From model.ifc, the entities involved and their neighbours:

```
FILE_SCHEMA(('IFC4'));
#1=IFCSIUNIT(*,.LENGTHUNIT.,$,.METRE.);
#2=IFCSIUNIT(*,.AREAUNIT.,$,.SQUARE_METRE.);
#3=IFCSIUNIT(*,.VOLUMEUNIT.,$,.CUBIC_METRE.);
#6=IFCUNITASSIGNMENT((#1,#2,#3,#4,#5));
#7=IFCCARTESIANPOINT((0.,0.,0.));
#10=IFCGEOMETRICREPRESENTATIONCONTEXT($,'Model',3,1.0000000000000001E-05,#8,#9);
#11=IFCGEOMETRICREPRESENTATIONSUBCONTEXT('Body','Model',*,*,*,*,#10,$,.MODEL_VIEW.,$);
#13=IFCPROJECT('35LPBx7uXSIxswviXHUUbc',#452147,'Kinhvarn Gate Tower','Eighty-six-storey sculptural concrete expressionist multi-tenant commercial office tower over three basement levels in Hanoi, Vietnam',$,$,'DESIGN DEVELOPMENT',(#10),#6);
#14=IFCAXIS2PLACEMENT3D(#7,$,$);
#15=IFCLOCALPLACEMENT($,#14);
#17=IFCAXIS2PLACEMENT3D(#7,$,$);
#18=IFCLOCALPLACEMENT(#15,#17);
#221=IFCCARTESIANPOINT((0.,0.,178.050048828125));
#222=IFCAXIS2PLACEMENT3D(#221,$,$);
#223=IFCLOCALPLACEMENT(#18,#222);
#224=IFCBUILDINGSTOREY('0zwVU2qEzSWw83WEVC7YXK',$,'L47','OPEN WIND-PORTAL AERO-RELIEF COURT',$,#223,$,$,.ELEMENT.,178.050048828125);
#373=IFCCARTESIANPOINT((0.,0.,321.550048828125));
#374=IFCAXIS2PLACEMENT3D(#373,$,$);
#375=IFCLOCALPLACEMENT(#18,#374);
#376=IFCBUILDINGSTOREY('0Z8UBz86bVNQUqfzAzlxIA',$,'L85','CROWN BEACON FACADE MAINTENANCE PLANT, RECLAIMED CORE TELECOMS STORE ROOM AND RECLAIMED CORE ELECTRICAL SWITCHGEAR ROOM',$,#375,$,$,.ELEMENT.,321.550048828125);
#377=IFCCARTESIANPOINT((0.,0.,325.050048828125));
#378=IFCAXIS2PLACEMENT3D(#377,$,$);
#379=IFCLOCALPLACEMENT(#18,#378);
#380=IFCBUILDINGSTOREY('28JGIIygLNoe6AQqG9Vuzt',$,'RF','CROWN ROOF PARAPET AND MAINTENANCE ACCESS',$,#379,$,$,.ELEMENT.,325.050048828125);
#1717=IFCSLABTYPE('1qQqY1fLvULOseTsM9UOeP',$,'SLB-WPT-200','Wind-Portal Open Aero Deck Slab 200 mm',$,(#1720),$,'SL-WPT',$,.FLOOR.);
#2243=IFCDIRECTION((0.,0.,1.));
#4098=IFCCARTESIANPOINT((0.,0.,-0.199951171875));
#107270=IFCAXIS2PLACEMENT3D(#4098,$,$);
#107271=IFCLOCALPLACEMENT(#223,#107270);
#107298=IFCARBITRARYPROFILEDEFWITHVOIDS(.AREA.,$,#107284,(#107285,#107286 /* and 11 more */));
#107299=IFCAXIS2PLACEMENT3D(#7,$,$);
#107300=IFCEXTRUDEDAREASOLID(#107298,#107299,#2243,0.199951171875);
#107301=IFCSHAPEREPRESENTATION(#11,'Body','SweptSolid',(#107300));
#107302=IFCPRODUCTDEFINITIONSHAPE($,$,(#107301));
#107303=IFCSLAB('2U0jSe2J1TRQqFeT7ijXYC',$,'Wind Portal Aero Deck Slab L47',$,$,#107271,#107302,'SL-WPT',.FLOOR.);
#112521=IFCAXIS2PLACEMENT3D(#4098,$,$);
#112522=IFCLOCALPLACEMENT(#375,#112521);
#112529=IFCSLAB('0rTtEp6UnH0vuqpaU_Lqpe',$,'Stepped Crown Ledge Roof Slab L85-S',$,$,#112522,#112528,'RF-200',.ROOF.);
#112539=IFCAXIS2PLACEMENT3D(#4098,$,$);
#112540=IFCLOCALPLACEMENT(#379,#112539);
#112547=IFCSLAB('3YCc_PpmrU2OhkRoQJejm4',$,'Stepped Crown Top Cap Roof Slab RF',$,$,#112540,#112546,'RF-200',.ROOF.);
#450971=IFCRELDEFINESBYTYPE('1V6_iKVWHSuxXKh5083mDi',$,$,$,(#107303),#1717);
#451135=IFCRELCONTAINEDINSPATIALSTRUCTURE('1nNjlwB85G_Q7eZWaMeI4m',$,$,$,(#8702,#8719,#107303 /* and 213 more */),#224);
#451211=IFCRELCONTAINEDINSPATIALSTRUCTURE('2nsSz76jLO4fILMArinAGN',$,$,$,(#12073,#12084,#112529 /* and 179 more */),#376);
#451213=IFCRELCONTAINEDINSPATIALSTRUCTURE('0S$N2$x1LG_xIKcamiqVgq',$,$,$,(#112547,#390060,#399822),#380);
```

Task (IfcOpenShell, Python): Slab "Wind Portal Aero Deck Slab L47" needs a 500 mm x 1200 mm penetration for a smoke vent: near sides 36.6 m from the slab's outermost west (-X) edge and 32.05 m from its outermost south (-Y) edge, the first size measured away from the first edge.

```python
import numpy as np
import ifcopenshell
import ifcopenshell.api.feature
import ifcopenshell.api.geometry
import ifcopenshell.api.root
import ifcopenshell.geom
import ifcopenshell.util.placement
import ifcopenshell.util.representation
import ifcopenshell.util.shape
import ifcopenshell.util.unit

model = ifcopenshell.open("model.ifc")
unit_scale = ifcopenshell.util.unit.calculate_unit_scale(model)
settings = ifcopenshell.geom.settings()


def volume(element):
    """Net volume in cubic metres, openings subtracted."""
    shape = ifcopenshell.geom.create_shape(settings, element)
    return ifcopenshell.util.shape.get_volume(shape.geometry)


slab = model.by_guid("2U0jSe2J1TRQqFeT7ijXYC")
before = volume(slab)

# Extent in the slab's own axes, in metres. The edges named are its -X and -Y sides.
slab_shape = ifcopenshell.geom.create_shape(settings, slab)
vertices = ifcopenshell.util.shape.get_vertices(slab_shape.geometry)
x_min, y_min, bottom = vertices.min(axis=0)
top = vertices[:, 2].max()

opening = ifcopenshell.api.root.create_entity(model, ifc_class="IfcOpeningElement", name="Smoke vent opening", predefined_type="OPENING")
context = ifcopenshell.util.representation.get_context(model, "Model", "Body", "MODEL_VIEW")
width, depth = 0.5, 1.2
outline = [(0.0, 0.0), (width, 0.0), (width, depth), (0.0, depth), (0.0, 0.0)]
# Overshoot both faces by 50 mm so the cut is clean.
shape = ifcopenshell.api.geometry.add_slab_representation(
    model, context=context, depth=top - bottom + 0.1, polyline=outline
)
ifcopenshell.api.geometry.assign_representation(model, product=opening, representation=shape)

matrix = ifcopenshell.util.placement.get_local_placement(slab.ObjectPlacement)
matrix[:, 3] = matrix @ np.append(np.array([x_min + 36.6, y_min + 32.05, bottom - 0.05]) / unit_scale, 1.0)
ifcopenshell.api.geometry.edit_object_placement(model, product=opening, matrix=matrix, is_si=False)
ifcopenshell.api.feature.add_feature(model, feature=opening, element=slab)

after = volume(slab)

print(f"slab volume {before:.3f} -> {after:.3f} m3")

model.write("model_edited.ifc")
```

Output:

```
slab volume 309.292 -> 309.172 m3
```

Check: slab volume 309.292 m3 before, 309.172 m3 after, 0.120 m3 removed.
